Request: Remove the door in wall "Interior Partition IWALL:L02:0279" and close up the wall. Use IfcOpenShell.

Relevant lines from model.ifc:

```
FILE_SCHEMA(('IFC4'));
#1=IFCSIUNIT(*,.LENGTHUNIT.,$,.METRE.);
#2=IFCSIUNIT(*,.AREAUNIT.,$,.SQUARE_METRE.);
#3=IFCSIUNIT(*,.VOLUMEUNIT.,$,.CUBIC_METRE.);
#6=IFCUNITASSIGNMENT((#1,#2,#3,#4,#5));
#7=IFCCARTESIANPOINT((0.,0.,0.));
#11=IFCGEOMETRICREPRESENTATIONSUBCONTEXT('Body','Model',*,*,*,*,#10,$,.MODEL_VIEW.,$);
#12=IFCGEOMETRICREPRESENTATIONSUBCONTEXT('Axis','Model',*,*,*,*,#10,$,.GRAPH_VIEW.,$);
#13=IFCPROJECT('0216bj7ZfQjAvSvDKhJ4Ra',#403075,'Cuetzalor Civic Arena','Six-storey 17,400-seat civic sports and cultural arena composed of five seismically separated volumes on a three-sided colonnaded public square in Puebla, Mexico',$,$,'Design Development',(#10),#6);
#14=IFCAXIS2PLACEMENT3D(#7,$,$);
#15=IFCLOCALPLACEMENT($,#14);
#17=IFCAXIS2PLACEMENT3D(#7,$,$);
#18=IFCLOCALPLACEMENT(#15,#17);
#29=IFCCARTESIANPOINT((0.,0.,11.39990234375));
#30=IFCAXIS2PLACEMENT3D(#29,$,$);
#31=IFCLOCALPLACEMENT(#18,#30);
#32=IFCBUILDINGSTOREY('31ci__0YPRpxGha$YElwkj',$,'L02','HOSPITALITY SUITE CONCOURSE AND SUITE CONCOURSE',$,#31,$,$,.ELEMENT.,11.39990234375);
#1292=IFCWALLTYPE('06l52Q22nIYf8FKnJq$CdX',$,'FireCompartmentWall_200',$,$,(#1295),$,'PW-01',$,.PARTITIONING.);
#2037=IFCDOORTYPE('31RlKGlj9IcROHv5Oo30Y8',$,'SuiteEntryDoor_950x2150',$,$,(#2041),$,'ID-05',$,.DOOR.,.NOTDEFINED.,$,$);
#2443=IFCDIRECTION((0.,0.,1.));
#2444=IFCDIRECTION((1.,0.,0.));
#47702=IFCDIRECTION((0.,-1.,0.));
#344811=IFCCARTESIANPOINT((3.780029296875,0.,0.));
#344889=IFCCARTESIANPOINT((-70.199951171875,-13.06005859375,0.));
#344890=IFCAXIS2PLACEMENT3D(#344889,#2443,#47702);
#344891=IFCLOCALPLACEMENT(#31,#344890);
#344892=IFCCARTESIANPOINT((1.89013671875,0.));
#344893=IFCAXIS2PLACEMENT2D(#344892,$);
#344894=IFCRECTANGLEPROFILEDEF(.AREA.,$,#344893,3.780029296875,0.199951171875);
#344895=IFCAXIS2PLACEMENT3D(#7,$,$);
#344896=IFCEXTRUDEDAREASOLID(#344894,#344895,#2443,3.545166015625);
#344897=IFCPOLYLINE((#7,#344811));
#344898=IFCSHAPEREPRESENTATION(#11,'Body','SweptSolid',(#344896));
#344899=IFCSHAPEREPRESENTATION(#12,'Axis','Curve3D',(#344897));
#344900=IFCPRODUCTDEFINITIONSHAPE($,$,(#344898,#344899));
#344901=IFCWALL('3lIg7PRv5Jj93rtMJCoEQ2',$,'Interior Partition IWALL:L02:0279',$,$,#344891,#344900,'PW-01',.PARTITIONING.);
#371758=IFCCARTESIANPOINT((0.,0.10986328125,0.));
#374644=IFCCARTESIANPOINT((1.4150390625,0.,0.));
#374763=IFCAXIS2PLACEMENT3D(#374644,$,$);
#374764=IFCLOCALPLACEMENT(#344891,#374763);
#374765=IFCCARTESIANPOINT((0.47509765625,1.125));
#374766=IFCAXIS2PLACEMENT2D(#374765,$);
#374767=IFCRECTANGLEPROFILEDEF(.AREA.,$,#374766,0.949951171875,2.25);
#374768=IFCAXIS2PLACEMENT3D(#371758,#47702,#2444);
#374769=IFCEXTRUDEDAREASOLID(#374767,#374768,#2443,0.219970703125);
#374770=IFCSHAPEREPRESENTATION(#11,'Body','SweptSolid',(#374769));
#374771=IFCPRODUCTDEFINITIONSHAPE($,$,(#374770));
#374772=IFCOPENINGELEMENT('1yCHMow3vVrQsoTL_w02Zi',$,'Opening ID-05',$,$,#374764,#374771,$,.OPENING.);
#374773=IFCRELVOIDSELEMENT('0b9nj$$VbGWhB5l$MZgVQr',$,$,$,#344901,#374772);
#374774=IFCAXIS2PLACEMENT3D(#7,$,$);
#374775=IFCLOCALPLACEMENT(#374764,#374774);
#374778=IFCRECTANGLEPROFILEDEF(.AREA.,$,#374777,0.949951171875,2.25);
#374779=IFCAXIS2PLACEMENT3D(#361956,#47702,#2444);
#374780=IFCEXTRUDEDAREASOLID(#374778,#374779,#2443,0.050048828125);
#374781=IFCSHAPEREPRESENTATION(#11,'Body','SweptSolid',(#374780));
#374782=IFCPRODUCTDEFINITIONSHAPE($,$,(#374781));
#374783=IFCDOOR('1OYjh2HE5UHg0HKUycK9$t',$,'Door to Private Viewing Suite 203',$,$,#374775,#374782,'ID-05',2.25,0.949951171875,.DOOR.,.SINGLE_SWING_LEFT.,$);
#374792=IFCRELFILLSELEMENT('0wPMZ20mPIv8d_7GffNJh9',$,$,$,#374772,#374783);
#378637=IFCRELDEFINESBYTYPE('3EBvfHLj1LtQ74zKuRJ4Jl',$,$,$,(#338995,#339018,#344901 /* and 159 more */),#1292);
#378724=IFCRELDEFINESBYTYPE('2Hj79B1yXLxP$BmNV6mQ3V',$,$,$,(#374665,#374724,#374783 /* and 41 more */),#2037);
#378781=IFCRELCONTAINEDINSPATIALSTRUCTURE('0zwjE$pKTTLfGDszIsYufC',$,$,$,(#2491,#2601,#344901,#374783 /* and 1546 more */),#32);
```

```python
import ifcopenshell
import ifcopenshell.api.feature
import ifcopenshell.api.root
import ifcopenshell.geom
import ifcopenshell.util.shape

model = ifcopenshell.open("model.ifc")
settings = ifcopenshell.geom.settings()


def volume(element):
    """Net volume in cubic metres, openings subtracted."""
    shape = ifcopenshell.geom.create_shape(settings, element)
    return ifcopenshell.util.shape.get_volume(shape.geometry)


door = model.by_id(374783)
opening = door.FillsVoids[0].RelatingOpeningElement
wall = opening.VoidsElements[0].RelatingBuildingElement
before = volume(wall)

ifcopenshell.api.root.remove_product(model, product=door)
ifcopenshell.api.feature.remove_feature(model, feature=opening)

after = volume(wall)

print(f"wall volume {before:.3f} -> {after:.3f} m3")

model.write("model_v2.ifc")
```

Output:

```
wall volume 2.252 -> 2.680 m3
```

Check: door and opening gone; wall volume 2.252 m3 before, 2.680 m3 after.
